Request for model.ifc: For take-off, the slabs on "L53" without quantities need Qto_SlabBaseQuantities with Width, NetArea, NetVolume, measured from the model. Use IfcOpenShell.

First a look at what the model holds.

```python
import ifcopenshell
import ifcopenshell.util.element
import ifcopenshell.util.unit

model = ifcopenshell.open("model.ifc")
print(model.schema)
for unit_type in ("LENGTHUNIT", "AREAUNIT", "VOLUMEUNIT"):
    print(unit_type, ifcopenshell.util.unit.calculate_unit_scale(model, unit_type))
storey = next(s for s in model.by_type("IfcBuildingStorey") if s.Name == "L53")
slabs = [e for e in ifcopenshell.util.element.get_decomposition(storey) if e.is_a("IfcSlab")]
for e in sorted(slabs, key=lambda e: e.id()):
    print(e.id(), e.is_a(), e.Name, list(ifcopenshell.util.element.get_psets(e, qtos_only=True)), sep=" | ")
```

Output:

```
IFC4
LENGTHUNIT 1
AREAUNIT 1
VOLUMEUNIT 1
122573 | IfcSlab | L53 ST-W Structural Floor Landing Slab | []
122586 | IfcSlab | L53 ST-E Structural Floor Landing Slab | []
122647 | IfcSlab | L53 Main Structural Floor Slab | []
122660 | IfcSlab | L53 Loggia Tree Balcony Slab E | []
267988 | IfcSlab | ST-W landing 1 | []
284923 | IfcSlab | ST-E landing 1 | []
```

```python
import ifcopenshell
import ifcopenshell.api.pset
import ifcopenshell.geom
import ifcopenshell.util.element
import ifcopenshell.util.shape
import ifcopenshell.util.unit

model = ifcopenshell.open("model.ifc")
unit_scale = ifcopenshell.util.unit.calculate_unit_scale(model)
area_scale = ifcopenshell.util.unit.calculate_unit_scale(model, "AREAUNIT")
volume_scale = ifcopenshell.util.unit.calculate_unit_scale(model, "VOLUMEUNIT")
settings = ifcopenshell.geom.settings()

storey = next(s for s in model.by_type("IfcBuildingStorey") if s.Name == "L53")
slabs = [e for e in ifcopenshell.util.element.get_decomposition(storey) if e.is_a("IfcSlab")]

for e in sorted(slabs, key=lambda e: e.id()):
    if ifcopenshell.util.element.get_psets(e, qtos_only=True, should_inherit=False):
        continue
    # Geometry comes back in metres, in the element's own axes.
    shape = ifcopenshell.geom.create_shape(settings, e)
    values = {
        "Width": ifcopenshell.util.shape.get_z(shape.geometry) / unit_scale,
        "NetArea": ifcopenshell.util.shape.get_footprint_area(shape.geometry) / area_scale,
        "NetVolume": ifcopenshell.util.shape.get_volume(shape.geometry) / volume_scale,
    }
    qto = ifcopenshell.api.pset.add_qto(model, product=e, name="Qto_SlabBaseQuantities")
    ifcopenshell.api.pset.edit_qto(model, qto=qto, properties=values)
    print(e.id(), {k: round(v, 3) for k, v in values.items()})

model.write("model_edited.ifc")
```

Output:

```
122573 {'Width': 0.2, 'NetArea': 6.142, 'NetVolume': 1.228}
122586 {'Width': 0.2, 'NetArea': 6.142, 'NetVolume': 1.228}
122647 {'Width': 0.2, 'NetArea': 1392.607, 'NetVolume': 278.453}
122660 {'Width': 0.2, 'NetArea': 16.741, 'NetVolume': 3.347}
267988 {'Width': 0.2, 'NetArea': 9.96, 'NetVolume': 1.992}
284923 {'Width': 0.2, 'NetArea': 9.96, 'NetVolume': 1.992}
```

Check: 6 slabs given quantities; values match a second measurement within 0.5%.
